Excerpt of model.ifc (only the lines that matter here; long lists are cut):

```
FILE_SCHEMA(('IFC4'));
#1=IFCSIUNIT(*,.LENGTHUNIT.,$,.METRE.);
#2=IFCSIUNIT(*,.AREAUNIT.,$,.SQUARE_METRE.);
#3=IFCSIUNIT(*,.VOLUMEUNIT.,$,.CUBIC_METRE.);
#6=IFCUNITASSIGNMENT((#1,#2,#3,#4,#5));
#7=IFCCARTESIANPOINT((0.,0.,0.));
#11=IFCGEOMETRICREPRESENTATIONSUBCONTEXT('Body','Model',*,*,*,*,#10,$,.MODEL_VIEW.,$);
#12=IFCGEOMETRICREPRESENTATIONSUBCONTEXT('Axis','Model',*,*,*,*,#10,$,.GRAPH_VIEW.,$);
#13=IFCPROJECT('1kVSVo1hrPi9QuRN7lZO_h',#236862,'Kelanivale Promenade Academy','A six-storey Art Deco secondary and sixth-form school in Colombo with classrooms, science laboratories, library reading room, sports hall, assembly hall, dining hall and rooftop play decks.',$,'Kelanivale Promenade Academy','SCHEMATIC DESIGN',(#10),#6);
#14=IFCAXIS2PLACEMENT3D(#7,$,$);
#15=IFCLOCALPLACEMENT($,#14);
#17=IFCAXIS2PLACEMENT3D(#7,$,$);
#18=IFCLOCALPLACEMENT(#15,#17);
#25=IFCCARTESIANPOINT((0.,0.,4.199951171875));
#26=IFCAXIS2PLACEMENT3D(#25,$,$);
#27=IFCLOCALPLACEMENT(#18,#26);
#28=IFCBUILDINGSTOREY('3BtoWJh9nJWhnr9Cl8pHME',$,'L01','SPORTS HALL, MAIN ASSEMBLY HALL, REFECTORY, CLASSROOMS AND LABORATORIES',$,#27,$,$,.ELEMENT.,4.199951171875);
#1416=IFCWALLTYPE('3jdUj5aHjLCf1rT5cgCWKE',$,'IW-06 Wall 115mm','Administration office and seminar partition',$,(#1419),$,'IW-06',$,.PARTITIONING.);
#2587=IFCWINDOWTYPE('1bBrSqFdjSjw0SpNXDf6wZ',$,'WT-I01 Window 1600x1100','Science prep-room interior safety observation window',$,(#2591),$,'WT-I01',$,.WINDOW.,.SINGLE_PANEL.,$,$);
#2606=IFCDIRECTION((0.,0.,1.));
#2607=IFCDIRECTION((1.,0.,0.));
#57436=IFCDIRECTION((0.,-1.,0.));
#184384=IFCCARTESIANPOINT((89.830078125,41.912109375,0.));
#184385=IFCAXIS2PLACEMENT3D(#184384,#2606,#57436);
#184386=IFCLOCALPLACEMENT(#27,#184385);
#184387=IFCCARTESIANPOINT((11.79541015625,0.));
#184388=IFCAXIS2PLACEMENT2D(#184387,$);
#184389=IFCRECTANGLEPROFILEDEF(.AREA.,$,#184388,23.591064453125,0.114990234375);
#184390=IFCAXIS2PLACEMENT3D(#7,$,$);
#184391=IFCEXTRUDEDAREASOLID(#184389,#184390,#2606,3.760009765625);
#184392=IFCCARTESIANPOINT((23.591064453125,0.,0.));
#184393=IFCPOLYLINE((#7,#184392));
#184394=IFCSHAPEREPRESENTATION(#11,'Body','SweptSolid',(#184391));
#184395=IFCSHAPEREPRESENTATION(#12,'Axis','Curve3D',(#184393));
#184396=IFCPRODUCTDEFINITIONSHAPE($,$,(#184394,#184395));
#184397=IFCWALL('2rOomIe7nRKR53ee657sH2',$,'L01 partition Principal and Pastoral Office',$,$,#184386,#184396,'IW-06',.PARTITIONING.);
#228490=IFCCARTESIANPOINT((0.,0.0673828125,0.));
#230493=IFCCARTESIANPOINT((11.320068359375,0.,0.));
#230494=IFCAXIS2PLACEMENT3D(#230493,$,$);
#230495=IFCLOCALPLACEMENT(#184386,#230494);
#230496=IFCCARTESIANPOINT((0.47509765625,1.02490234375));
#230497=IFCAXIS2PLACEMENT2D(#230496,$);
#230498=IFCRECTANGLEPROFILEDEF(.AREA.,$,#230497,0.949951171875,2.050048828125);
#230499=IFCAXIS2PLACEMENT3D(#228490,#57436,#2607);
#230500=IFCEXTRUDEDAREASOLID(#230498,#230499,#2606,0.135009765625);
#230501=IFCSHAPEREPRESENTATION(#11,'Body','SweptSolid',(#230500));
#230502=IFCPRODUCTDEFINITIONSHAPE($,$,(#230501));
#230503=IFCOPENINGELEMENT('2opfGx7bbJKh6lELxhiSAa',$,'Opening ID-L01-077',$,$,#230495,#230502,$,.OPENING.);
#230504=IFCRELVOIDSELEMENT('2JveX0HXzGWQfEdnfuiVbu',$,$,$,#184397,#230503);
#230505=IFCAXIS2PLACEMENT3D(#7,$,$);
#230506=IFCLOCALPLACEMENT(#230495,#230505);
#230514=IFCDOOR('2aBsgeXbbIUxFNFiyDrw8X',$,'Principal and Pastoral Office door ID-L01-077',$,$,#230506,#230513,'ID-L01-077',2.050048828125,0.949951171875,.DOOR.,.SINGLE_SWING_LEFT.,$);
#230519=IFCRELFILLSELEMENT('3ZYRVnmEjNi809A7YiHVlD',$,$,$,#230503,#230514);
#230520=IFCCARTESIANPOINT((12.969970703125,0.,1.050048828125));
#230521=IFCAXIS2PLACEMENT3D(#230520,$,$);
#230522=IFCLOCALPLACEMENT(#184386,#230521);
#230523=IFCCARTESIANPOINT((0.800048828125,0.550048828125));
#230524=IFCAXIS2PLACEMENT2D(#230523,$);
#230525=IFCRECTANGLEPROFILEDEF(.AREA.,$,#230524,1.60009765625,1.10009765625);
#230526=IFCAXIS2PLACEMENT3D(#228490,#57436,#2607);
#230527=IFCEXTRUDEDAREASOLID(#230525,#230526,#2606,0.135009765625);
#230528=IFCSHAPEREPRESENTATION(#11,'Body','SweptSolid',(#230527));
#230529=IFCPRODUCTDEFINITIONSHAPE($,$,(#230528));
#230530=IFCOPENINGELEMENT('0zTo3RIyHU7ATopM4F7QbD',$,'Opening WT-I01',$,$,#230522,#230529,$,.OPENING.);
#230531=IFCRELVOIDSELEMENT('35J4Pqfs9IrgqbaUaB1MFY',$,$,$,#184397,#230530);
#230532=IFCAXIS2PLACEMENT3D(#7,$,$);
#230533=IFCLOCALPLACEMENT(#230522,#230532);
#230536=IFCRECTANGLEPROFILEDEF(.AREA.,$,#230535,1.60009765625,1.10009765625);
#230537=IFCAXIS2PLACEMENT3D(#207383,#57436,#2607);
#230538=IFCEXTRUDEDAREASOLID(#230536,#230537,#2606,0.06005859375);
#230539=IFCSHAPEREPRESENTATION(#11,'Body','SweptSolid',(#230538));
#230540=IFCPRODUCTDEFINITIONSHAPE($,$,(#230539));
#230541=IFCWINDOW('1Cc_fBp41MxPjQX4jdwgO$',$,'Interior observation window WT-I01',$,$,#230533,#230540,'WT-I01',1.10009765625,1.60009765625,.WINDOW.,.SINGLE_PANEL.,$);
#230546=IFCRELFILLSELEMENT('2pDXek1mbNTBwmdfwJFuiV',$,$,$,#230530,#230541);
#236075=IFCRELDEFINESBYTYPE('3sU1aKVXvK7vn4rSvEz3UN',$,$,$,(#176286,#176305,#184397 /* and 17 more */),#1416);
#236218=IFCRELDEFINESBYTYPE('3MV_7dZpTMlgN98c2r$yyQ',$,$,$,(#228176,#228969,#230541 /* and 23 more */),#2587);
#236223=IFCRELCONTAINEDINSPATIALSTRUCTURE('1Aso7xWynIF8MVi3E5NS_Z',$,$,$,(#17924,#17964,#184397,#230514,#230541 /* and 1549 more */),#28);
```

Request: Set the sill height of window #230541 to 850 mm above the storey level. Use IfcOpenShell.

```python
import numpy as np
import ifcopenshell
import ifcopenshell.api.geometry
import ifcopenshell.geom
import ifcopenshell.util.element
import ifcopenshell.util.placement
import ifcopenshell.util.shape
import ifcopenshell.util.unit

model = ifcopenshell.open("model.ifc")
unit_scale = ifcopenshell.util.unit.calculate_unit_scale(model)

window = model.by_guid("1Cc_fBp41MxPjQX4jdwgO$")
opening = window.FillsVoids[0].RelatingOpeningElement
storey = ifcopenshell.util.element.get_container(window, ifc_class="IfcBuildingStorey")
level = ifcopenshell.util.placement.get_local_placement(storey.ObjectPlacement)[2, 3]

# The opening's origin need not be at the sill, so measure its lowest point.
shape = ifcopenshell.geom.create_shape(ifcopenshell.geom.settings(), opening)
bottom = ifcopenshell.util.shape.get_shape_bottom_elevation(shape, shape.geometry) / unit_scale
dz = level + 0.85 / unit_scale - bottom

shift = np.array([0.0, 0.0, dz])
# The window is placed relative to its opening, so it follows when the opening moves.
matrix = ifcopenshell.util.placement.get_local_placement(opening.ObjectPlacement)
matrix[:3, 3] += shift
ifcopenshell.api.geometry.edit_object_placement(
    model, product=opening, matrix=matrix, is_si=False, should_transform_children=True
)

print(f"moved by {dz * unit_scale:+.3f} m")

model.write("model_rev.ifc")
```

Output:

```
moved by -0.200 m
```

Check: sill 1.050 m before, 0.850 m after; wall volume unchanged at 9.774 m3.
